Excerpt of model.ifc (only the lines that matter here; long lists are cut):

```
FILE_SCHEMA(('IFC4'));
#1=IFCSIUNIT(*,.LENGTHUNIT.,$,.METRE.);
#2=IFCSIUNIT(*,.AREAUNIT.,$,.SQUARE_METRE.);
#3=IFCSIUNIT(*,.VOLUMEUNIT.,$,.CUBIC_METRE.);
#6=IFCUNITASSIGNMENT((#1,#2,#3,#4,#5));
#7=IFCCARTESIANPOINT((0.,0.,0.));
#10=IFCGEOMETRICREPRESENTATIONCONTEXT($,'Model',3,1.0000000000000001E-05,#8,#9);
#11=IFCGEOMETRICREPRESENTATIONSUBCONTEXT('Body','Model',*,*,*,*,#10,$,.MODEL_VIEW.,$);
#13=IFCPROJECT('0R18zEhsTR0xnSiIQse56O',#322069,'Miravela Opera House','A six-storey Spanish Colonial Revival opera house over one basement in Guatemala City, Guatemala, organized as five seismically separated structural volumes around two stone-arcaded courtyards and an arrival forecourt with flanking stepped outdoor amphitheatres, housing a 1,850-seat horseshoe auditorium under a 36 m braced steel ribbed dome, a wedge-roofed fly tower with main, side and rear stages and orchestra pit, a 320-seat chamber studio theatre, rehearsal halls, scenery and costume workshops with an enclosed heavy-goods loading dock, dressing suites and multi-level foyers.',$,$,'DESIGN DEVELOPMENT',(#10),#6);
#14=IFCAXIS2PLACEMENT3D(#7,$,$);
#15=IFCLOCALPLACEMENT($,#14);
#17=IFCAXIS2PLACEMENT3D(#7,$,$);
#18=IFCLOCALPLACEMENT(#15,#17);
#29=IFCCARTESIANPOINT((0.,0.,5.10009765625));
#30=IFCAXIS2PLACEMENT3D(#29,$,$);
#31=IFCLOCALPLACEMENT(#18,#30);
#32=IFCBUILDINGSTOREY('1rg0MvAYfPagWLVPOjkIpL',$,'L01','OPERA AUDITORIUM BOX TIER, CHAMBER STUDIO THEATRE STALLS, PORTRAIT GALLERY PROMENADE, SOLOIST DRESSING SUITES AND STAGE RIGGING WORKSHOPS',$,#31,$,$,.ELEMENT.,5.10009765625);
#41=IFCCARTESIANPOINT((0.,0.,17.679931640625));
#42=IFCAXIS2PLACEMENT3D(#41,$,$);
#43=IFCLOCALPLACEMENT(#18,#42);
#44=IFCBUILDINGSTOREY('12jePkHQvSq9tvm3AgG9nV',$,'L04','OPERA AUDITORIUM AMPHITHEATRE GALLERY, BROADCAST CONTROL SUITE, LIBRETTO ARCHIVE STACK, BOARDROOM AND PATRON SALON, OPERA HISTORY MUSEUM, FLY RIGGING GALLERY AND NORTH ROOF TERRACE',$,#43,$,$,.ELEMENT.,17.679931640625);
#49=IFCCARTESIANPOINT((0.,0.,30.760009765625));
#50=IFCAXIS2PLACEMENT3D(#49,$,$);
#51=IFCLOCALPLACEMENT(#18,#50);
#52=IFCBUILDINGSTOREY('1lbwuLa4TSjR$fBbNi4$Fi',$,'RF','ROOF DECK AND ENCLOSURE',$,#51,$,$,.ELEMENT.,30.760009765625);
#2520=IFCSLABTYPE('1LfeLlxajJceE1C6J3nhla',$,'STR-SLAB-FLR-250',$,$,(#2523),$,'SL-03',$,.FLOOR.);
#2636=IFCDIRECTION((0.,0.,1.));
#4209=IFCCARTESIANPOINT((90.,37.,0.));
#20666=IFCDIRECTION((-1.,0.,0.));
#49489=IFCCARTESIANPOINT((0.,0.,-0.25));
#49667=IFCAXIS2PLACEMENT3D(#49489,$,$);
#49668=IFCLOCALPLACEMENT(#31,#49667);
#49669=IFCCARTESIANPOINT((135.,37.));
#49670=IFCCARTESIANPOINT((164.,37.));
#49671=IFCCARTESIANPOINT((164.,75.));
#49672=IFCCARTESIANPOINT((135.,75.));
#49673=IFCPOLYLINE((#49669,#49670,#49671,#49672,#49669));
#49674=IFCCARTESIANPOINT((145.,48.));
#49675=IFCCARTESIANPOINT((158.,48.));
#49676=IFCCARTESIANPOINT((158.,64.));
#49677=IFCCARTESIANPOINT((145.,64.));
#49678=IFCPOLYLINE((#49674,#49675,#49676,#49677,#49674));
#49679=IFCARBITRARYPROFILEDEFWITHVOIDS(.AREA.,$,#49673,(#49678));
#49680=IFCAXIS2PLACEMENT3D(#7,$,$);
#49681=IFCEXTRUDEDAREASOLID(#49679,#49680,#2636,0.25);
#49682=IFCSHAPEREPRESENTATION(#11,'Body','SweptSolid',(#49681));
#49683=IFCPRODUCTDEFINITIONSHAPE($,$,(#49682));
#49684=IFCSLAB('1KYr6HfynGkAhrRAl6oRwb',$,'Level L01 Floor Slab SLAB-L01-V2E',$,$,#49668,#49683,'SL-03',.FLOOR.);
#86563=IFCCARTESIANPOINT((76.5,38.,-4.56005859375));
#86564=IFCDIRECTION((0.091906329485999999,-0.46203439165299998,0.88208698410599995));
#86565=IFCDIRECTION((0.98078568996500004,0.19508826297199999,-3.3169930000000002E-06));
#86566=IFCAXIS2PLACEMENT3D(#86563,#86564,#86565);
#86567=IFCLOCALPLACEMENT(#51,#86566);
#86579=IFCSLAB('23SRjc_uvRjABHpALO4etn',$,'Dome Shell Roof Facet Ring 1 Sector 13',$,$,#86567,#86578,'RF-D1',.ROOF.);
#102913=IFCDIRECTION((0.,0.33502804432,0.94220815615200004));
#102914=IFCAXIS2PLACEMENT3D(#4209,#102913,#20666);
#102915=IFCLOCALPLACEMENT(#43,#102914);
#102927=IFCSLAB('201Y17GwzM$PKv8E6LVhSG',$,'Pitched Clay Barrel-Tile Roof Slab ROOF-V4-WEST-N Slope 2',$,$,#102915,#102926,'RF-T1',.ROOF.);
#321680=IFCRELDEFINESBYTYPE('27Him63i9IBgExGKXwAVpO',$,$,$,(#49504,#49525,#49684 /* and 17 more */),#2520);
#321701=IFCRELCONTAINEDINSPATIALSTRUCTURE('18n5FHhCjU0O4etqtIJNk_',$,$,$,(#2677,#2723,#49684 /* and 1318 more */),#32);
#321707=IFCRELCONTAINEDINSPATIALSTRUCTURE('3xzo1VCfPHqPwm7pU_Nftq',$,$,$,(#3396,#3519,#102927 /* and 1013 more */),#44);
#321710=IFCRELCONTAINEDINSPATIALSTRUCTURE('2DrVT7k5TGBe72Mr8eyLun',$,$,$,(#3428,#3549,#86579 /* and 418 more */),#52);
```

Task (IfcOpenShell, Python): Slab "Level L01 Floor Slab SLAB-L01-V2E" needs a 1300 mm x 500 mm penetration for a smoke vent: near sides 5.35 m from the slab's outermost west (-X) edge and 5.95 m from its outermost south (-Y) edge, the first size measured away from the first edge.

```python
import numpy as np
import ifcopenshell
import ifcopenshell.api.feature
import ifcopenshell.api.geometry
import ifcopenshell.api.root
import ifcopenshell.geom
import ifcopenshell.util.placement
import ifcopenshell.util.representation
import ifcopenshell.util.shape
import ifcopenshell.util.unit

model = ifcopenshell.open("model.ifc")
unit_scale = ifcopenshell.util.unit.calculate_unit_scale(model)
settings = ifcopenshell.geom.settings()


def volume(element):
    """Net volume in cubic metres, openings subtracted."""
    shape = ifcopenshell.geom.create_shape(settings, element)
    return ifcopenshell.util.shape.get_volume(shape.geometry)


slab = model.by_guid("1KYr6HfynGkAhrRAl6oRwb")
before = volume(slab)

# Extent in the slab's own axes, in metres. The edges named are its -X and -Y sides.
slab_shape = ifcopenshell.geom.create_shape(settings, slab)
vertices = ifcopenshell.util.shape.get_vertices(slab_shape.geometry)
x_min, y_min, bottom = vertices.min(axis=0)
top = vertices[:, 2].max()

opening = ifcopenshell.api.root.create_entity(model, ifc_class="IfcOpeningElement", name="Smoke vent opening", predefined_type="OPENING")
context = ifcopenshell.util.representation.get_context(model, "Model", "Body", "MODEL_VIEW")
width, depth = 1.3, 0.5
outline = [(0.0, 0.0), (width, 0.0), (width, depth), (0.0, depth), (0.0, 0.0)]
# Overshoot both faces by 50 mm so the cut is clean.
shape = ifcopenshell.api.geometry.add_slab_representation(
    model, context=context, depth=top - bottom + 0.1, polyline=outline
)
ifcopenshell.api.geometry.assign_representation(model, product=opening, representation=shape)

matrix = ifcopenshell.util.placement.get_local_placement(slab.ObjectPlacement)
matrix[:, 3] = matrix @ np.append(np.array([x_min + 5.35, y_min + 5.95, bottom - 0.05]) / unit_scale, 1.0)
ifcopenshell.api.geometry.edit_object_placement(model, product=opening, matrix=matrix, is_si=False)
ifcopenshell.api.feature.add_feature(model, feature=opening, element=slab)

after = volume(slab)

print(f"slab volume {before:.3f} -> {after:.3f} m3")

model.write("model_v2.ifc")
```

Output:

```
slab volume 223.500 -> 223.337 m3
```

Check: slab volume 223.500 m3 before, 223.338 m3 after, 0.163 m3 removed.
